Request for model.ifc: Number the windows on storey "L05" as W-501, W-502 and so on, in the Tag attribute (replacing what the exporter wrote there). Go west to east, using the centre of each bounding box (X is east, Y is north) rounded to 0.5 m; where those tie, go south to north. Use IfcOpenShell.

First a look at what the model holds.

```python
import ifcopenshell
import ifcopenshell.util.element
import ifcopenshell.util.placement

model = ifcopenshell.open("model.ifc")
print(model.schema)
storey = next(s for s in model.by_type("IfcBuildingStorey") if s.Name == "L05")
windows = [e for e in ifcopenshell.util.element.get_decomposition(storey) if e.is_a("IfcWindow")]
for e in sorted(windows, key=lambda e: e.id()):
    origin = ifcopenshell.util.placement.get_local_placement(e.ObjectPlacement)[:3, 3]
    print(e.id(), e.Tag, e.Name, origin.round(2) + 0.0, sep=" | ")
```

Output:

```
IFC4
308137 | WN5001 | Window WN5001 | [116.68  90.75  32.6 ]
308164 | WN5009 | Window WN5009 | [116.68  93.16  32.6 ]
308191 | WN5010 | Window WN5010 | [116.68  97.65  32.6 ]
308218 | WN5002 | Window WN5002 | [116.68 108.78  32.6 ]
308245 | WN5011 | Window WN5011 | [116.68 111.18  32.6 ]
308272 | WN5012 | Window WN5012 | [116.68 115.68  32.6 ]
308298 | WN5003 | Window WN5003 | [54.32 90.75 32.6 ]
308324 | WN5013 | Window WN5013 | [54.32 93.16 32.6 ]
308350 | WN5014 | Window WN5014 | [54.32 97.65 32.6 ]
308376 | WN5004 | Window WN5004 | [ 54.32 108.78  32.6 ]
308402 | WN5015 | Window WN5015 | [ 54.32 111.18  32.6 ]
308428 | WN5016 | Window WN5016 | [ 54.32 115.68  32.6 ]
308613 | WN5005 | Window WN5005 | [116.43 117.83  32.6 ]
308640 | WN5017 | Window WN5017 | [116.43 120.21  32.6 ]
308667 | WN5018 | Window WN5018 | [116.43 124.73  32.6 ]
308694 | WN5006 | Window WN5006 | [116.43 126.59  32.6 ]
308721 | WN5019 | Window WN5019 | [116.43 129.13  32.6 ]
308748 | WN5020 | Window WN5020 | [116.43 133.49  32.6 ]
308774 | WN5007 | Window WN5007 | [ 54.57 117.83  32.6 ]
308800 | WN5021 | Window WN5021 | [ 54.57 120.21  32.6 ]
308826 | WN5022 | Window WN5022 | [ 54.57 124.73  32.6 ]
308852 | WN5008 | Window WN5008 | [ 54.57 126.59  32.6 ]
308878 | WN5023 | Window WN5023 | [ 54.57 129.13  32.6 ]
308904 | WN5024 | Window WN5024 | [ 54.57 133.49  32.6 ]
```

```python
import ifcopenshell
import ifcopenshell.geom
import ifcopenshell.util.element
import ifcopenshell.util.shape

model = ifcopenshell.open("model.ifc")
settings = ifcopenshell.geom.settings()
settings.set("use-world-coords", True)


def centre(element):
    shape = ifcopenshell.geom.create_shape(settings, element)
    return ifcopenshell.util.shape.get_bbox_centroid(shape.geometry)


storey = next(s for s in model.by_type("IfcBuildingStorey") if s.Name == "L05")
windows = [e for e in ifcopenshell.util.element.get_decomposition(storey) if e.is_a("IfcWindow")]

# Insertion points can sit at a corner or the storey origin, so sort by the geometry (in metres).
centres = {e: centre(e) for e in windows}
windows.sort(key=lambda e: (round(centres[e][0] / 0.5), centres[e][1]))

for i, e in enumerate(windows, start=1):
    number = f"W-5{i:02d}"
    e.Tag = number
    print(e.id(), number)

model.write("model_edited.ifc")
```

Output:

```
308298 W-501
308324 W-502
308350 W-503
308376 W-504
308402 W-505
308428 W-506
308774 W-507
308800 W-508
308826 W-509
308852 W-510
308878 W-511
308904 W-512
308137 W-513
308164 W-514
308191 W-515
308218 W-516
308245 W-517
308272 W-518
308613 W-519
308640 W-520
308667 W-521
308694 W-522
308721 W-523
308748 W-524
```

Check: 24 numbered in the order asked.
